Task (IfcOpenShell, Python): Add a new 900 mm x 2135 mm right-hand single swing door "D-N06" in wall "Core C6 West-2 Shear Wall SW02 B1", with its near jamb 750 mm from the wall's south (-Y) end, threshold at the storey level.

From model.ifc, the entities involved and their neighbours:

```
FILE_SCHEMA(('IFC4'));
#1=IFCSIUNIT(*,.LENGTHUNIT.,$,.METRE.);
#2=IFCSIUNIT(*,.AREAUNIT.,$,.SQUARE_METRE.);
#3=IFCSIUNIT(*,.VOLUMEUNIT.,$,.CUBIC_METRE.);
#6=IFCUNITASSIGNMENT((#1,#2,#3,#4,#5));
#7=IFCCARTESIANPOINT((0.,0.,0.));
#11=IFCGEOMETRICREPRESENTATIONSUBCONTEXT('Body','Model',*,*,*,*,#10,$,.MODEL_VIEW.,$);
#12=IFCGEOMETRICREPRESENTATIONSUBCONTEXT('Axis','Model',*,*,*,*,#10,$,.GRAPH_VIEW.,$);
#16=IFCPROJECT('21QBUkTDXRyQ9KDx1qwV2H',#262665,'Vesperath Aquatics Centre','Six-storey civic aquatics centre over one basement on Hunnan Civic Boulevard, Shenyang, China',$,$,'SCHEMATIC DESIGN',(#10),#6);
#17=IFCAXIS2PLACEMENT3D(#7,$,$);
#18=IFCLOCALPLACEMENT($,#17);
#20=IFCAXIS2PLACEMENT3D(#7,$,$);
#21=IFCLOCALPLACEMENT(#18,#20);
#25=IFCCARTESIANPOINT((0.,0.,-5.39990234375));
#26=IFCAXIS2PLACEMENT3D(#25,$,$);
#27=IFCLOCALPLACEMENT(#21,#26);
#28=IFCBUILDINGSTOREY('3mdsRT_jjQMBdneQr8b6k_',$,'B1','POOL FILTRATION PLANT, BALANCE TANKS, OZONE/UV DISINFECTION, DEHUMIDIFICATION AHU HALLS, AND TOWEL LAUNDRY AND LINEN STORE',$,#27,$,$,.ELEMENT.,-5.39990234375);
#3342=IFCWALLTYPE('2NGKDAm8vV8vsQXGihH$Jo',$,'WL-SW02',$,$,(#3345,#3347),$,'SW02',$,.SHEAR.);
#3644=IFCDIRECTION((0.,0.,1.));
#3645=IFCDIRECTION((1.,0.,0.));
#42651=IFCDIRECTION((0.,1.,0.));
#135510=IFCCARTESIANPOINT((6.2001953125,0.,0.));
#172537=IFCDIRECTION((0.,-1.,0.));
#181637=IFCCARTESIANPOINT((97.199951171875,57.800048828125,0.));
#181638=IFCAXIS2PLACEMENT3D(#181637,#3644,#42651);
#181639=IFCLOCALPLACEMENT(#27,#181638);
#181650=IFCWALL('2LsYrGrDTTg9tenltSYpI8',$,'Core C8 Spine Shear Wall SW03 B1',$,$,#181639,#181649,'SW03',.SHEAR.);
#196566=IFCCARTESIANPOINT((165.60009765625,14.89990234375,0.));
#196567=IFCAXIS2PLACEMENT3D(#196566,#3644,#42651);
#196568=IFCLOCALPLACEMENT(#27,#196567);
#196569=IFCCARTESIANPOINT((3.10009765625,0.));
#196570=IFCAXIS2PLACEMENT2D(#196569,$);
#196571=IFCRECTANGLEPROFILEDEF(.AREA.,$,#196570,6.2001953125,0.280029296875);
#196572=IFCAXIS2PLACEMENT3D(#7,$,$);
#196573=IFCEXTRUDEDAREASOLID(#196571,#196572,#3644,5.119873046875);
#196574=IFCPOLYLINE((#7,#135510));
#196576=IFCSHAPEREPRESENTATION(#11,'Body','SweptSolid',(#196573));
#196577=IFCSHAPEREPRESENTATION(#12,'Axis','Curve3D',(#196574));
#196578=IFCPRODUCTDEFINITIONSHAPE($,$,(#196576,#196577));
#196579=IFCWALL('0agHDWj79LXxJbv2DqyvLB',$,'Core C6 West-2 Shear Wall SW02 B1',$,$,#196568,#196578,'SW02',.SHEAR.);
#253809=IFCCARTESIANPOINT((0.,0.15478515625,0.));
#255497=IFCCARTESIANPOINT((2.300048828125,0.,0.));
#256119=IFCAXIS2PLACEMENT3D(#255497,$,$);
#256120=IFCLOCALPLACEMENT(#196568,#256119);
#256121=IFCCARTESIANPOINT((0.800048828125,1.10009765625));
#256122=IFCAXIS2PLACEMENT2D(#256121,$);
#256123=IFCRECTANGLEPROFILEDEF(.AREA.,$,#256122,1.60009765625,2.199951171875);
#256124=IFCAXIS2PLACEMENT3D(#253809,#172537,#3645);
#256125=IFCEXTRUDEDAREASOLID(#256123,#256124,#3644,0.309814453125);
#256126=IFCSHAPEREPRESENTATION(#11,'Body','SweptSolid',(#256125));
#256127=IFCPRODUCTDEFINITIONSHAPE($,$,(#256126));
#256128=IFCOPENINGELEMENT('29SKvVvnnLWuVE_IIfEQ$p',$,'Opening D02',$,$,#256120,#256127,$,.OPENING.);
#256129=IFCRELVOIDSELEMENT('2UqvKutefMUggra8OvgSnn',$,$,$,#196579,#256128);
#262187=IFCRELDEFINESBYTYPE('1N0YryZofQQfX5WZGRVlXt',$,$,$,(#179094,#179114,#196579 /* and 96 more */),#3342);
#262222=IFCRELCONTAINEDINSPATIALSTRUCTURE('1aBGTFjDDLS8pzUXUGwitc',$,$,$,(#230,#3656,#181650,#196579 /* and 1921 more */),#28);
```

```python
import numpy as np
import ifcopenshell
import ifcopenshell.api.feature
import ifcopenshell.api.geometry
import ifcopenshell.api.root
import ifcopenshell.api.spatial
import ifcopenshell.geom
import ifcopenshell.util.element
import ifcopenshell.util.placement
import ifcopenshell.util.representation
import ifcopenshell.util.shape
import ifcopenshell.util.unit

model = ifcopenshell.open("model.ifc")
unit_scale = ifcopenshell.util.unit.calculate_unit_scale(model)
settings = ifcopenshell.geom.settings()


def volume(element):
    """Net volume in cubic metres, openings subtracted."""
    shape = ifcopenshell.geom.create_shape(settings, element)
    return ifcopenshell.util.shape.get_volume(shape.geometry)


wall = model.by_guid("0agHDWj79LXxJbv2DqyvLB")
storey = ifcopenshell.util.element.get_container(wall, ifc_class="IfcBuildingStorey")
context = ifcopenshell.util.representation.get_context(model, "Model", "Body", "MODEL_VIEW")
before = volume(wall)

width, height, from_end, sill = 0.9, 2.135, 0.75, 0.0  # metres

# The wall runs along its own X axis, and the end named is its -X end.
wall_shape = ifcopenshell.geom.create_shape(settings, wall)
x, y, z = ifcopenshell.util.shape.get_vertices(wall_shape.geometry).T
start = x.min() + from_end
face, thickness = float(y.min()), float(y.max() - y.min())
wall_matrix = ifcopenshell.util.placement.get_local_placement(wall.ObjectPlacement)
level = ifcopenshell.util.placement.get_local_placement(storey.ObjectPlacement)[2, 3]


def in_wall(x, y):
    """Placement at x, y metres in the wall's axes, at sill height."""
    matrix = wall_matrix.copy()
    matrix[:, 3] = wall_matrix @ np.array([x / unit_scale, y / unit_scale, 0.0, 1.0])
    matrix[2, 3] = level + sill / unit_scale
    return matrix


# Opening: a box that overshoots both wall faces by 50 mm.
opening = ifcopenshell.api.root.create_entity(model, ifc_class="IfcOpeningElement", predefined_type="OPENING")
box = ifcopenshell.api.geometry.add_wall_representation(
    model, context=context, length=width, height=height, thickness=thickness + 0.1
)
ifcopenshell.api.geometry.assign_representation(model, product=opening, representation=box)
ifcopenshell.api.geometry.edit_object_placement(model, product=opening, matrix=in_wall(start, face - 0.05), is_si=False)
ifcopenshell.api.feature.add_feature(model, feature=opening, element=wall)

door = ifcopenshell.api.root.create_entity(model, ifc_class="IfcDoor", name="D-N06", predefined_type="DOOR")
door.OverallWidth, door.OverallHeight = width / unit_scale, height / unit_scale
door.OperationType = "SINGLE_SWING_RIGHT"
body = ifcopenshell.api.geometry.add_door_representation(
    model,
    context=context,
    overall_width=door.OverallWidth,
    overall_height=door.OverallHeight,
    operation_type="SINGLE_SWING_RIGHT",
    lining_properties={"LiningDepth": thickness / unit_scale, "ThresholdDepth": thickness / unit_scale},
)
ifcopenshell.api.geometry.assign_representation(model, product=door, representation=body)
ifcopenshell.api.spatial.assign_container(model, products=[door], relating_structure=storey)
ifcopenshell.api.feature.add_filling(model, opening=opening, element=door)

# The lining spans the wall, so the door starts at the wall face.
ifcopenshell.api.geometry.edit_object_placement(model, product=door, matrix=in_wall(start, face), is_si=False)

after = volume(wall)

print(f"wall volume {before:.3f} -> {after:.3f} m3")

model.write("model_updated.ifc")
```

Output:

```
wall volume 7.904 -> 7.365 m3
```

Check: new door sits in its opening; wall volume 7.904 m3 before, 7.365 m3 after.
